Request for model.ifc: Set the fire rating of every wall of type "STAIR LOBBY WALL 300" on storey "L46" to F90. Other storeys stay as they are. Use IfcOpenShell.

First a look at what the model holds.

```python
import ifcopenshell
import ifcopenshell.util.element

model = ifcopenshell.open("model.ifc")
print(model.schema)
storey = next(s for s in model.by_type("IfcBuildingStorey") if s.Name == "L46")
walls = [e for e in ifcopenshell.util.element.get_decomposition(storey) if e.is_a("IfcWall")]
seen = {}
for e in walls:
    element_type = ifcopenshell.util.element.get_type(e)
    key = (element_type.Name if element_type != e and element_type else None, ifcopenshell.util.element.get_pset(e, "Pset_WallCommon", "FireRating"))
    seen[key] = seen.get(key, 0) + 1
for (name, value), count in sorted(seen.items(), key=str):
    print(count, "x", name, "|", value)
```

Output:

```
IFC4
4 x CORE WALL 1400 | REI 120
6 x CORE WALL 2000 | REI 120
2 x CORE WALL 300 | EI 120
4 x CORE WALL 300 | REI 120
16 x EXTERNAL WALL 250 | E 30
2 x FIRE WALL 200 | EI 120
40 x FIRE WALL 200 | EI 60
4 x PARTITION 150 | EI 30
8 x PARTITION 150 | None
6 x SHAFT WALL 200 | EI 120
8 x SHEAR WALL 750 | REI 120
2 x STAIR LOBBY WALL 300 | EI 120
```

```python
import ifcopenshell
import ifcopenshell.api.pset
import ifcopenshell.util.element

model = ifcopenshell.open("model.ifc")

storey = next(s for s in model.by_type("IfcBuildingStorey") if s.Name == "L46")
walls = [e for e in ifcopenshell.util.element.get_decomposition(storey) if e.is_a("IfcWall")]

count = 0
for e in walls:
    element_type = ifcopenshell.util.element.get_type(e)
    if element_type in (None, e) or element_type.Name != "STAIR LOBBY WALL 300":
        continue
    found = ifcopenshell.util.element.get_pset(e, "Pset_WallCommon", should_inherit=False)
    if found:
        pset = model.by_id(found["id"])
        if len(ifcopenshell.util.element.get_elements_by_pset(pset)) > 1:
            pset = ifcopenshell.api.pset.unshare_pset(model, products=[e], pset=pset)[0]
    else:
        pset = ifcopenshell.api.pset.add_pset(model, product=e, name="Pset_WallCommon")
    ifcopenshell.api.pset.edit_pset(model, pset=pset, properties={"FireRating": "F90"})
    count += 1

print(count, "walls updated")

model.write("model_v2.ifc")
```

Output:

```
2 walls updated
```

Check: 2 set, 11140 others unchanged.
